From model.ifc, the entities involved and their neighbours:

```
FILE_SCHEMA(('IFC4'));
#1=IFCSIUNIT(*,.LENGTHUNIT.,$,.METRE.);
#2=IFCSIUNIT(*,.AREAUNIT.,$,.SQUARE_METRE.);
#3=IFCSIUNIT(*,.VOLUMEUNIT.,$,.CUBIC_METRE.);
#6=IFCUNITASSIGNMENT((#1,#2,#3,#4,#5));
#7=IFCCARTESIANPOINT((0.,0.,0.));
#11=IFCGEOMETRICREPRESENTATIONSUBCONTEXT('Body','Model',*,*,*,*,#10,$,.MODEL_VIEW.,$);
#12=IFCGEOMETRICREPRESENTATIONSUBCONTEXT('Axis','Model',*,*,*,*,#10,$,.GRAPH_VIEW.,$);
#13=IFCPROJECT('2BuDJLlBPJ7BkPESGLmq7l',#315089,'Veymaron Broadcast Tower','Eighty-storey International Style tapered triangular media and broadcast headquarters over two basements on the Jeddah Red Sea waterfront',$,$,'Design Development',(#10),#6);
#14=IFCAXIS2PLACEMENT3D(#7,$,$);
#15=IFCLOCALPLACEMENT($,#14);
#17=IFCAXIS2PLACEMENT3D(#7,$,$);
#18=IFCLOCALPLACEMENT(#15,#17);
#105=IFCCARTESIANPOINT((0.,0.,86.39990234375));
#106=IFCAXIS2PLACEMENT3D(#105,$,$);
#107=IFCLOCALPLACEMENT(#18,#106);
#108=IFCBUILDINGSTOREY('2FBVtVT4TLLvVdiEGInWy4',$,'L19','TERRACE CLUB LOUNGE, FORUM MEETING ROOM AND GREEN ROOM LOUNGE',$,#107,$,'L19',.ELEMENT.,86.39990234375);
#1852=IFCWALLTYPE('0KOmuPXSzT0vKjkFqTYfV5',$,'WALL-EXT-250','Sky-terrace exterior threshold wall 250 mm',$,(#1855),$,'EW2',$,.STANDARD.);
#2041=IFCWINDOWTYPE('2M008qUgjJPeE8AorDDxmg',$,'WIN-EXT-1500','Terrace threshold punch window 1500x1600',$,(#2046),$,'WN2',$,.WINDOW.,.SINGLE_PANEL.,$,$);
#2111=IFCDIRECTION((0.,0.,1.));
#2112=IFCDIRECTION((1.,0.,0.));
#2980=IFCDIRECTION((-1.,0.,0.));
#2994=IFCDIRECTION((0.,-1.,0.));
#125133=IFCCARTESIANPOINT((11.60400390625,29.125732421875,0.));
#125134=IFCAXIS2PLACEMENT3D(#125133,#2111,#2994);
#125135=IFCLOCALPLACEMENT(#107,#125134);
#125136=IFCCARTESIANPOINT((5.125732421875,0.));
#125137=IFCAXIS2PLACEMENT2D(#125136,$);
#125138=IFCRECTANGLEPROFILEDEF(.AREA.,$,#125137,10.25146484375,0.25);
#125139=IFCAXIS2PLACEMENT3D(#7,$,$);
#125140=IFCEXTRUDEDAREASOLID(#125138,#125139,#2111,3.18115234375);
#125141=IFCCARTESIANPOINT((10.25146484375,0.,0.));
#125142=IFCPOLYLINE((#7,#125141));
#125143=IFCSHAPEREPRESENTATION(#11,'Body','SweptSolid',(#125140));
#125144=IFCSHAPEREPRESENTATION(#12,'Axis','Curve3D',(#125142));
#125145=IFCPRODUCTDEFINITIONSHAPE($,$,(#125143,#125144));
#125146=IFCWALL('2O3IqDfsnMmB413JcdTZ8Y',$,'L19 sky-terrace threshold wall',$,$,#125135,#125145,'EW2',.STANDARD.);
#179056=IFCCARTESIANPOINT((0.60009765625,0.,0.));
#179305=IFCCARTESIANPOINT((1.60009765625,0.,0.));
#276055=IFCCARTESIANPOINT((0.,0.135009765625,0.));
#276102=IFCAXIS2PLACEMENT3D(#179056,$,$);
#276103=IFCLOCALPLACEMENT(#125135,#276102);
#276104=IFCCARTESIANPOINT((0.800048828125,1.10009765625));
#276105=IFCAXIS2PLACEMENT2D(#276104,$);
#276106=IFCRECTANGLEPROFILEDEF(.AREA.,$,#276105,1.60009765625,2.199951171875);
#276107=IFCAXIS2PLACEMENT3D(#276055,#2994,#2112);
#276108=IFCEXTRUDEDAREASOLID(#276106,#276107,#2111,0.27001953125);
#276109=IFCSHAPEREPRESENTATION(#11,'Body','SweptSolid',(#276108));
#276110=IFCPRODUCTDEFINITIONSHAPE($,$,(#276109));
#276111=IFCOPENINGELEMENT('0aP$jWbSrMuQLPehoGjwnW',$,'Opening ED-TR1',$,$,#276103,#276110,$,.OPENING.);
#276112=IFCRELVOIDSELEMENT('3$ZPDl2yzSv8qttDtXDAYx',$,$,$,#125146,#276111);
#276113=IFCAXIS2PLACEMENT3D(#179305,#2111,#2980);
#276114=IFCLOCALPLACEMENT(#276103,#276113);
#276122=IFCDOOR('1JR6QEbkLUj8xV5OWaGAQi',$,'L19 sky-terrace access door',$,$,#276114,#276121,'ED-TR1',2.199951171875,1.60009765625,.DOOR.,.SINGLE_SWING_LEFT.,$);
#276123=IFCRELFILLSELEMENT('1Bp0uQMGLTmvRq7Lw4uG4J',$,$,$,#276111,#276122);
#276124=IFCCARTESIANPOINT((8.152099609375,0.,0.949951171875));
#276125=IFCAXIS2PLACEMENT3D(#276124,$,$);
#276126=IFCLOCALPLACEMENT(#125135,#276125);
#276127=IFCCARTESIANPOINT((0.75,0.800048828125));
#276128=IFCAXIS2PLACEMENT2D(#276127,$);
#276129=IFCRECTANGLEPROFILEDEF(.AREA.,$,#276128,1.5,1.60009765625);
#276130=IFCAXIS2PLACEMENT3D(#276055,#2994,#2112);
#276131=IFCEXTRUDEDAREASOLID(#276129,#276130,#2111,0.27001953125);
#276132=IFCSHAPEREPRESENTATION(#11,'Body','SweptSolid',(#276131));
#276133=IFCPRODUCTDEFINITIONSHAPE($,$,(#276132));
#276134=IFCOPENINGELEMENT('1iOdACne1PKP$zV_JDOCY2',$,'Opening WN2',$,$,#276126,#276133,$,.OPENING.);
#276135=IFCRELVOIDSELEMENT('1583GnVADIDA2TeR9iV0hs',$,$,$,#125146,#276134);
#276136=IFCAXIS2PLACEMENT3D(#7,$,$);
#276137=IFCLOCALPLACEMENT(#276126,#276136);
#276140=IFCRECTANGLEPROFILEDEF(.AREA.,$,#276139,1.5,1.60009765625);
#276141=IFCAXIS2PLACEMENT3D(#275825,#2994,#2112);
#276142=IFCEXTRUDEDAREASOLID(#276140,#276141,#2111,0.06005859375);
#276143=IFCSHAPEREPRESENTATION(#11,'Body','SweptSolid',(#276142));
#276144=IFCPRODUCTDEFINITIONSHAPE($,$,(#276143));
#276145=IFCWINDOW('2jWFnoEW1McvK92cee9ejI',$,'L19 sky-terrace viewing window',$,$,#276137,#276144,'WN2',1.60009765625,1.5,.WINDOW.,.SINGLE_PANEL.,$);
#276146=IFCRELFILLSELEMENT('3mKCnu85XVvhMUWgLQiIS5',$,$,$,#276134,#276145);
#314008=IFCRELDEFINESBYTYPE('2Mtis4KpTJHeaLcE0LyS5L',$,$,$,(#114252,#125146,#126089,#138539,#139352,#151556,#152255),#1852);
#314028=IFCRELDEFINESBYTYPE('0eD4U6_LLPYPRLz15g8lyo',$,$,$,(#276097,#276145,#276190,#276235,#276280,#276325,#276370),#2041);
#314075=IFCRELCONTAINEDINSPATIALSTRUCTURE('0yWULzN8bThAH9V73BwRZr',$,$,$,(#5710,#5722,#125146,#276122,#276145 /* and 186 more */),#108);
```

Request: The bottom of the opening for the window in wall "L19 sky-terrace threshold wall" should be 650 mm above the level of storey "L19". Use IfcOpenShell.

```python
import numpy as np
import ifcopenshell
import ifcopenshell.api.geometry
import ifcopenshell.geom
import ifcopenshell.util.element
import ifcopenshell.util.placement
import ifcopenshell.util.shape
import ifcopenshell.util.unit

model = ifcopenshell.open("model.ifc")
unit_scale = ifcopenshell.util.unit.calculate_unit_scale(model)

window = model.by_guid("2jWFnoEW1McvK92cee9ejI")
opening = window.FillsVoids[0].RelatingOpeningElement
storey = ifcopenshell.util.element.get_container(window, ifc_class="IfcBuildingStorey")
level = ifcopenshell.util.placement.get_local_placement(storey.ObjectPlacement)[2, 3]

# The opening's origin need not be at the sill, so measure its lowest point.
shape = ifcopenshell.geom.create_shape(ifcopenshell.geom.settings(), opening)
bottom = ifcopenshell.util.shape.get_shape_bottom_elevation(shape, shape.geometry) / unit_scale
dz = level + 0.65 / unit_scale - bottom

shift = np.array([0.0, 0.0, dz])
# The window is placed relative to its opening, so it follows when the opening moves.
matrix = ifcopenshell.util.placement.get_local_placement(opening.ObjectPlacement)
matrix[:3, 3] += shift
ifcopenshell.api.geometry.edit_object_placement(
    model, product=opening, matrix=matrix, is_si=False, should_transform_children=True
)

print(f"moved by {dz * unit_scale:+.3f} m")

model.write("model_updated.ifc")
```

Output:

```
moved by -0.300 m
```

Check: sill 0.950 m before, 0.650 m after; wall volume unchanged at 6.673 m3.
